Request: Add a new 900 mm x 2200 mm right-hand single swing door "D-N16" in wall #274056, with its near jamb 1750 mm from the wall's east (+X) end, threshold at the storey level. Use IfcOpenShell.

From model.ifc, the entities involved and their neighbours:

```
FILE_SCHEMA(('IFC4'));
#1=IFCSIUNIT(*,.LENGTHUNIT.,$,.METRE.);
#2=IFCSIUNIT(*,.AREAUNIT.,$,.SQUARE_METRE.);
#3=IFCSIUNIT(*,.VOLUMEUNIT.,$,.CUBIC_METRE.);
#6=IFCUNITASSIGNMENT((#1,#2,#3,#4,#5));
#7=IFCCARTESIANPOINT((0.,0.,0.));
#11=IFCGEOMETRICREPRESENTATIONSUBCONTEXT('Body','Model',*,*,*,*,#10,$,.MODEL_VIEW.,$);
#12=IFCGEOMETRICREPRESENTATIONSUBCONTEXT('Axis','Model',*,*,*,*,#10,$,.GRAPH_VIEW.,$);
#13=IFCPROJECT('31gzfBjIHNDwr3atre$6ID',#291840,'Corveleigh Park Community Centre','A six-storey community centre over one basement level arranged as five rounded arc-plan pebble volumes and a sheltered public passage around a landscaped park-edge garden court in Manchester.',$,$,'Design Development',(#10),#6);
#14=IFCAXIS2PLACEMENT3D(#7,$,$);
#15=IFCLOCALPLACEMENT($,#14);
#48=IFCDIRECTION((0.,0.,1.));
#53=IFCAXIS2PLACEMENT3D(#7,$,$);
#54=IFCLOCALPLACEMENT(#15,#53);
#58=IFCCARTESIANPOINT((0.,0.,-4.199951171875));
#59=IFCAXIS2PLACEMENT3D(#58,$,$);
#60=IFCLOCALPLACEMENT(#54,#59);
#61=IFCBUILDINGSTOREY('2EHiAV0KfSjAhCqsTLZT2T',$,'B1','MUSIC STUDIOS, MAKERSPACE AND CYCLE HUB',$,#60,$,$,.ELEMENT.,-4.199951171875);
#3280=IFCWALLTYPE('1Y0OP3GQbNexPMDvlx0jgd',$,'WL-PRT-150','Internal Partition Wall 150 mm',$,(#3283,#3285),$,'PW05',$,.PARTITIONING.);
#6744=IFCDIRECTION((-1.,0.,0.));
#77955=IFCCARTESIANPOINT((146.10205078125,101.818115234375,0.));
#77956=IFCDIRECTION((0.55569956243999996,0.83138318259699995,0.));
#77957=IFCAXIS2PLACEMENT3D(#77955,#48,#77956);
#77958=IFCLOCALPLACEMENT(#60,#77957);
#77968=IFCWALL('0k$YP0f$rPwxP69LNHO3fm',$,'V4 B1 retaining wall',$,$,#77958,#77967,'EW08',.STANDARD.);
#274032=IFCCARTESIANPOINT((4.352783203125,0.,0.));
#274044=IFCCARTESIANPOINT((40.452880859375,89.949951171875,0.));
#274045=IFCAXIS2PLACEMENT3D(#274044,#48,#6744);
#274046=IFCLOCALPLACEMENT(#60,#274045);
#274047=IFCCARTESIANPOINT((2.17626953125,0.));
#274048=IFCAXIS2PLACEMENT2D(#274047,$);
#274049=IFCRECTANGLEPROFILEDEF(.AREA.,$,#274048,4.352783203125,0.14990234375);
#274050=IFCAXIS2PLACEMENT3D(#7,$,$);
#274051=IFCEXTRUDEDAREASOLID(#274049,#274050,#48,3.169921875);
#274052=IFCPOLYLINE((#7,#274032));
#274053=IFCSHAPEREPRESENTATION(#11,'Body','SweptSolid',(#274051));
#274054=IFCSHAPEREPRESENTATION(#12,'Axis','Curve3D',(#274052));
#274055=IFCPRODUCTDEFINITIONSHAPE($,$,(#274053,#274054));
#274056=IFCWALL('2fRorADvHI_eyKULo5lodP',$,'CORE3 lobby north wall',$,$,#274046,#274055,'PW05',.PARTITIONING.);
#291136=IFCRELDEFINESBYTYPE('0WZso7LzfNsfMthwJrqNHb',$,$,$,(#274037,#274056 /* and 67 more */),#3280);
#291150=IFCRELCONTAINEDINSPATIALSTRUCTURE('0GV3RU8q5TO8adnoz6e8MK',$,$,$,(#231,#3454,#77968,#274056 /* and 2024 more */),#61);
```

```python
import numpy as np
import ifcopenshell
import ifcopenshell.api.feature
import ifcopenshell.api.geometry
import ifcopenshell.api.root
import ifcopenshell.api.spatial
import ifcopenshell.geom
import ifcopenshell.util.element
import ifcopenshell.util.placement
import ifcopenshell.util.representation
import ifcopenshell.util.shape
import ifcopenshell.util.unit

model = ifcopenshell.open("model.ifc")
unit_scale = ifcopenshell.util.unit.calculate_unit_scale(model)
settings = ifcopenshell.geom.settings()


def volume(element):
    """Net volume in cubic metres, openings subtracted."""
    shape = ifcopenshell.geom.create_shape(settings, element)
    return ifcopenshell.util.shape.get_volume(shape.geometry)


wall = model.by_guid("2fRorADvHI_eyKULo5lodP")
storey = ifcopenshell.util.element.get_container(wall, ifc_class="IfcBuildingStorey")
context = ifcopenshell.util.representation.get_context(model, "Model", "Body", "MODEL_VIEW")
before = volume(wall)

width, height, from_end, sill = 0.9, 2.2, 1.75, 0.0  # metres

# The wall runs along its own X axis, and the end named is its -X end.
wall_shape = ifcopenshell.geom.create_shape(settings, wall)
x, y, z = ifcopenshell.util.shape.get_vertices(wall_shape.geometry).T
start = x.min() + from_end
face, thickness = float(y.min()), float(y.max() - y.min())
wall_matrix = ifcopenshell.util.placement.get_local_placement(wall.ObjectPlacement)
level = ifcopenshell.util.placement.get_local_placement(storey.ObjectPlacement)[2, 3]


def in_wall(x, y):
    """Placement at x, y metres in the wall's axes, at sill height."""
    matrix = wall_matrix.copy()
    matrix[:, 3] = wall_matrix @ np.array([x / unit_scale, y / unit_scale, 0.0, 1.0])
    matrix[2, 3] = level + sill / unit_scale
    return matrix


# Opening: a box that overshoots both wall faces by 50 mm.
opening = ifcopenshell.api.root.create_entity(model, ifc_class="IfcOpeningElement", predefined_type="OPENING")
box = ifcopenshell.api.geometry.add_wall_representation(
    model, context=context, length=width, height=height, thickness=thickness + 0.1
)
ifcopenshell.api.geometry.assign_representation(model, product=opening, representation=box)
ifcopenshell.api.geometry.edit_object_placement(model, product=opening, matrix=in_wall(start, face - 0.05), is_si=False)
ifcopenshell.api.feature.add_feature(model, feature=opening, element=wall)

door = ifcopenshell.api.root.create_entity(model, ifc_class="IfcDoor", name="D-N16", predefined_type="DOOR")
door.OverallWidth, door.OverallHeight = width / unit_scale, height / unit_scale
door.OperationType = "SINGLE_SWING_RIGHT"
body = ifcopenshell.api.geometry.add_door_representation(
    model,
    context=context,
    overall_width=door.OverallWidth,
    overall_height=door.OverallHeight,
    operation_type="SINGLE_SWING_RIGHT",
    lining_properties={"LiningDepth": thickness / unit_scale, "ThresholdDepth": thickness / unit_scale},
)
ifcopenshell.api.geometry.assign_representation(model, product=door, representation=body)
ifcopenshell.api.spatial.assign_container(model, products=[door], relating_structure=storey)
ifcopenshell.api.feature.add_filling(model, opening=opening, element=door)

# The lining spans the wall, so the door starts at the wall face.
ifcopenshell.api.geometry.edit_object_placement(model, product=door, matrix=in_wall(start, face), is_si=False)

after = volume(wall)

print(f"wall volume {before:.3f} -> {after:.3f} m3")

model.write("model_updated.ifc")
```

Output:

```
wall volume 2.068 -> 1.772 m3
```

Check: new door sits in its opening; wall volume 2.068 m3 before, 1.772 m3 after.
